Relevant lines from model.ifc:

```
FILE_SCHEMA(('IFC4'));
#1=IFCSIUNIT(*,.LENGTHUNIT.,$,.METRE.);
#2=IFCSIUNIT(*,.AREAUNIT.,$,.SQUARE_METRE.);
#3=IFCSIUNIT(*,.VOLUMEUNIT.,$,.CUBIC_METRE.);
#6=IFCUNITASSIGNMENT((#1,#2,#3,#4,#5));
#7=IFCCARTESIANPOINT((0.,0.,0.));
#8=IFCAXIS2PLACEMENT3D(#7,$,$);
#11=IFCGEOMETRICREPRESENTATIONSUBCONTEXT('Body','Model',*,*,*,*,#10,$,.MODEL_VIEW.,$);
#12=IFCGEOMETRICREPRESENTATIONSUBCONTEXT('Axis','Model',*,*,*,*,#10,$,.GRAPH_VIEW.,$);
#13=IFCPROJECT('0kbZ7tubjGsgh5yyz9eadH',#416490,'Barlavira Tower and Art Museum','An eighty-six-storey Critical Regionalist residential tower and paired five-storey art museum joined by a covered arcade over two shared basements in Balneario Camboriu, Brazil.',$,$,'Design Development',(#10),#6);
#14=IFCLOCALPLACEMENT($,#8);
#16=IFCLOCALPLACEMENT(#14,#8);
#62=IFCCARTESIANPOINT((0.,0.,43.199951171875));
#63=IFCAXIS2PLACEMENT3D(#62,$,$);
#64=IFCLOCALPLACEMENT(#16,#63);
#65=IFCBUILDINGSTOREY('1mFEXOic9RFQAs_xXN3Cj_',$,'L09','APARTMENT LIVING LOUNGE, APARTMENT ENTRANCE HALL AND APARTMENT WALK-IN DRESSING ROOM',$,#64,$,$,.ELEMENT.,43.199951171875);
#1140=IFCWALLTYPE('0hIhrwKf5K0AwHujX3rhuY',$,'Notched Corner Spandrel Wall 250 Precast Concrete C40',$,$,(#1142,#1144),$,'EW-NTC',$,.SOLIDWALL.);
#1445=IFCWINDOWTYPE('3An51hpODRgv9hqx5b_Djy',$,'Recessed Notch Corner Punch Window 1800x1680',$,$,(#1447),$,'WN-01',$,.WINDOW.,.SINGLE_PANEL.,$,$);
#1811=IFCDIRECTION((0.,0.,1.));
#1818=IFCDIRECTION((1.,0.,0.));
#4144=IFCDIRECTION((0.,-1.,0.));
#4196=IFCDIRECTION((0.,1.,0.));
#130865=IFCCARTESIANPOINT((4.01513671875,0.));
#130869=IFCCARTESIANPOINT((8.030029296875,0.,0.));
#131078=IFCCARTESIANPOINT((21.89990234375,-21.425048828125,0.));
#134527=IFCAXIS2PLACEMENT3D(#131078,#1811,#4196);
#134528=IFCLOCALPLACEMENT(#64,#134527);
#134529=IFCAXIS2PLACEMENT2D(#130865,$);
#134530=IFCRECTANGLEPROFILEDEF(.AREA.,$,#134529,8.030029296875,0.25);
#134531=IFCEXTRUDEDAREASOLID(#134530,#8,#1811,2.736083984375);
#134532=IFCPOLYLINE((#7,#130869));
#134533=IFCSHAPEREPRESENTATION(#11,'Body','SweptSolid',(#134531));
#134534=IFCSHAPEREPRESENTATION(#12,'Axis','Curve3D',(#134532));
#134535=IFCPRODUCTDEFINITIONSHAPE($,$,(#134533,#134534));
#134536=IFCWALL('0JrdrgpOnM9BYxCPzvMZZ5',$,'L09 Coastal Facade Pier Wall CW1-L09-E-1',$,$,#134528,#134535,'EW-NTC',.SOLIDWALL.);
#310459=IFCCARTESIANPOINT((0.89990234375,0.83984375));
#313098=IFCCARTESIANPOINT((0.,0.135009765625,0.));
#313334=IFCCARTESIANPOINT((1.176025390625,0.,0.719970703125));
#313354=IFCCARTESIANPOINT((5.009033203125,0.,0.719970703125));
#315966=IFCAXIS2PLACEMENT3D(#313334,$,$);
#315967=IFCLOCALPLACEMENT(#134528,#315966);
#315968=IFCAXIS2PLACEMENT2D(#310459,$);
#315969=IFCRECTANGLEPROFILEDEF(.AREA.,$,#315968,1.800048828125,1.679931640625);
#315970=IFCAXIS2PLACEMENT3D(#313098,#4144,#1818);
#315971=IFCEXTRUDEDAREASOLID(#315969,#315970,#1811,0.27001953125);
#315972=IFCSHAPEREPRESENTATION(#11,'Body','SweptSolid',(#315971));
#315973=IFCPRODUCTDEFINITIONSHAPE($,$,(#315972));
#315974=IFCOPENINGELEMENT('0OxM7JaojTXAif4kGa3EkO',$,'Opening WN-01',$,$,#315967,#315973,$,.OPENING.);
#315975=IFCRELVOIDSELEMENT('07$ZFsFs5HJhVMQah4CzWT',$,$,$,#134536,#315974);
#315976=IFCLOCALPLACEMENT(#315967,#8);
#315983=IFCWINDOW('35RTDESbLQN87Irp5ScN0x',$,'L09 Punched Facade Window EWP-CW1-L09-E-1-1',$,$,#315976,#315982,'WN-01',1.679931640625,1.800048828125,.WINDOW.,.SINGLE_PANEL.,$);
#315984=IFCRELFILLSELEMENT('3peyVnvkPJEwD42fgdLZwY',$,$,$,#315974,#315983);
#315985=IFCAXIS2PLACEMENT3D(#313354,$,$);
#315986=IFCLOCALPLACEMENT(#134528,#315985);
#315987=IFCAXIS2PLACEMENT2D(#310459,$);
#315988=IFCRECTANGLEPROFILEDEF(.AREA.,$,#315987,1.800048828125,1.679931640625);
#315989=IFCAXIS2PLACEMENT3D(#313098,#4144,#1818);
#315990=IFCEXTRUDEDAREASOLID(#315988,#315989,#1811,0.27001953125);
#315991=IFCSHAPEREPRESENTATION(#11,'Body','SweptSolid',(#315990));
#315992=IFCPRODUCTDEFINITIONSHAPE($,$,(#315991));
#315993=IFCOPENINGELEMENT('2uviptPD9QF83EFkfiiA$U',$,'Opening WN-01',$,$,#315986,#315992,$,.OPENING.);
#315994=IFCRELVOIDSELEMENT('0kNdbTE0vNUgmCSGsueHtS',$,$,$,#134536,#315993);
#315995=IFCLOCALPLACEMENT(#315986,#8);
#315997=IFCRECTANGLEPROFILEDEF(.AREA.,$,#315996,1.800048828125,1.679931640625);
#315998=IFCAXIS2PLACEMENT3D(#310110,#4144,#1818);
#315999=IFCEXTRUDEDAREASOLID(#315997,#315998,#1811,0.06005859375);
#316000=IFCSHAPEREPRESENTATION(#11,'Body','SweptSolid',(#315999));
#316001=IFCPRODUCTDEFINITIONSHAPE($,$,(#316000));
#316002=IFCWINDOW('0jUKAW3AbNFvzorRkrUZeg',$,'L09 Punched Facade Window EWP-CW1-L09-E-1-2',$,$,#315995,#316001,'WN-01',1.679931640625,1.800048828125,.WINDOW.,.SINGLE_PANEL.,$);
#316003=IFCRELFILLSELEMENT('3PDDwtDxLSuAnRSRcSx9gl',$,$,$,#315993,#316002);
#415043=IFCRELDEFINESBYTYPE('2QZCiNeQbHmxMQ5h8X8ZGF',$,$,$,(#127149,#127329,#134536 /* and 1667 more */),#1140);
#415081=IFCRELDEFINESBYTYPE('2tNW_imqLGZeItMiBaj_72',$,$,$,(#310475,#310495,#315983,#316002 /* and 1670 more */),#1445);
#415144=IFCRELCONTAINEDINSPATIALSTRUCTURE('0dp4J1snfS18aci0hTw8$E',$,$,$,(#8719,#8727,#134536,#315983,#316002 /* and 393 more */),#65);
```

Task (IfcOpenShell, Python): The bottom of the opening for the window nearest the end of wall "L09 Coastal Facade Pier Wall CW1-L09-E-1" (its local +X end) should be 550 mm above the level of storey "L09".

```python
import numpy as np
import ifcopenshell
import ifcopenshell.api.geometry
import ifcopenshell.geom
import ifcopenshell.util.element
import ifcopenshell.util.placement
import ifcopenshell.util.shape
import ifcopenshell.util.unit

model = ifcopenshell.open("model.ifc")
unit_scale = ifcopenshell.util.unit.calculate_unit_scale(model)

window = model.by_guid("0jUKAW3AbNFvzorRkrUZeg")
opening = window.FillsVoids[0].RelatingOpeningElement
storey = ifcopenshell.util.element.get_container(window, ifc_class="IfcBuildingStorey")
level = ifcopenshell.util.placement.get_local_placement(storey.ObjectPlacement)[2, 3]

# The opening's origin need not be at the sill, so measure its lowest point.
shape = ifcopenshell.geom.create_shape(ifcopenshell.geom.settings(), opening)
bottom = ifcopenshell.util.shape.get_shape_bottom_elevation(shape, shape.geometry) / unit_scale
dz = level + 0.55 / unit_scale - bottom

shift = np.array([0.0, 0.0, dz])
# The window is placed relative to its opening, so it follows when the opening moves.
matrix = ifcopenshell.util.placement.get_local_placement(opening.ObjectPlacement)
matrix[:3, 3] += shift
ifcopenshell.api.geometry.edit_object_placement(
    model, product=opening, matrix=matrix, is_si=False, should_transform_children=True
)

print(f"moved by {dz * unit_scale:+.3f} m")

model.write("model-out.ifc")
```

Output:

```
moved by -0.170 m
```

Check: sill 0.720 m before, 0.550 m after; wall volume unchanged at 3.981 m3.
